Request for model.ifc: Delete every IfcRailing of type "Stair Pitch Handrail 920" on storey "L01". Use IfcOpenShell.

First a look at what the model holds.

```python
import ifcopenshell
import ifcopenshell.util.element

model = ifcopenshell.open("model.ifc")
print(model.schema)
storey = next(s for s in model.by_type("IfcBuildingStorey") if s.Name == "L01")
railings = [e for e in ifcopenshell.util.element.get_decomposition(storey) if e.is_a("IfcRailing")]
seen = {}
for e in railings:
    element_type = ifcopenshell.util.element.get_type(e)
    name = element_type.Name if element_type not in (None, e) else None
    seen[name] = seen.get(name, 0) + 1
for name, count in sorted(seen.items(), key=str):
    print(count, "x", name)
```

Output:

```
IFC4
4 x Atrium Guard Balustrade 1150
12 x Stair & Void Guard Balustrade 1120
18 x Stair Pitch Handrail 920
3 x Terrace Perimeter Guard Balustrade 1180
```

```python
import ifcopenshell
import ifcopenshell.api.root
import ifcopenshell.util.element

model = ifcopenshell.open("model.ifc")

storey = next(s for s in model.by_type("IfcBuildingStorey") if s.Name == "L01")
railings = [e for e in ifcopenshell.util.element.get_decomposition(storey) if e.is_a("IfcRailing")]
targets = [e for e in railings if (t := ifcopenshell.util.element.get_type(e)) not in (None, e) and t.Name == "Stair Pitch Handrail 920"]

for e in targets:
    ifcopenshell.api.root.remove_product(model, product=e)
print(len(targets), "removed")

model.write("model-out.ifc")
```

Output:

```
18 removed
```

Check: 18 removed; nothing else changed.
